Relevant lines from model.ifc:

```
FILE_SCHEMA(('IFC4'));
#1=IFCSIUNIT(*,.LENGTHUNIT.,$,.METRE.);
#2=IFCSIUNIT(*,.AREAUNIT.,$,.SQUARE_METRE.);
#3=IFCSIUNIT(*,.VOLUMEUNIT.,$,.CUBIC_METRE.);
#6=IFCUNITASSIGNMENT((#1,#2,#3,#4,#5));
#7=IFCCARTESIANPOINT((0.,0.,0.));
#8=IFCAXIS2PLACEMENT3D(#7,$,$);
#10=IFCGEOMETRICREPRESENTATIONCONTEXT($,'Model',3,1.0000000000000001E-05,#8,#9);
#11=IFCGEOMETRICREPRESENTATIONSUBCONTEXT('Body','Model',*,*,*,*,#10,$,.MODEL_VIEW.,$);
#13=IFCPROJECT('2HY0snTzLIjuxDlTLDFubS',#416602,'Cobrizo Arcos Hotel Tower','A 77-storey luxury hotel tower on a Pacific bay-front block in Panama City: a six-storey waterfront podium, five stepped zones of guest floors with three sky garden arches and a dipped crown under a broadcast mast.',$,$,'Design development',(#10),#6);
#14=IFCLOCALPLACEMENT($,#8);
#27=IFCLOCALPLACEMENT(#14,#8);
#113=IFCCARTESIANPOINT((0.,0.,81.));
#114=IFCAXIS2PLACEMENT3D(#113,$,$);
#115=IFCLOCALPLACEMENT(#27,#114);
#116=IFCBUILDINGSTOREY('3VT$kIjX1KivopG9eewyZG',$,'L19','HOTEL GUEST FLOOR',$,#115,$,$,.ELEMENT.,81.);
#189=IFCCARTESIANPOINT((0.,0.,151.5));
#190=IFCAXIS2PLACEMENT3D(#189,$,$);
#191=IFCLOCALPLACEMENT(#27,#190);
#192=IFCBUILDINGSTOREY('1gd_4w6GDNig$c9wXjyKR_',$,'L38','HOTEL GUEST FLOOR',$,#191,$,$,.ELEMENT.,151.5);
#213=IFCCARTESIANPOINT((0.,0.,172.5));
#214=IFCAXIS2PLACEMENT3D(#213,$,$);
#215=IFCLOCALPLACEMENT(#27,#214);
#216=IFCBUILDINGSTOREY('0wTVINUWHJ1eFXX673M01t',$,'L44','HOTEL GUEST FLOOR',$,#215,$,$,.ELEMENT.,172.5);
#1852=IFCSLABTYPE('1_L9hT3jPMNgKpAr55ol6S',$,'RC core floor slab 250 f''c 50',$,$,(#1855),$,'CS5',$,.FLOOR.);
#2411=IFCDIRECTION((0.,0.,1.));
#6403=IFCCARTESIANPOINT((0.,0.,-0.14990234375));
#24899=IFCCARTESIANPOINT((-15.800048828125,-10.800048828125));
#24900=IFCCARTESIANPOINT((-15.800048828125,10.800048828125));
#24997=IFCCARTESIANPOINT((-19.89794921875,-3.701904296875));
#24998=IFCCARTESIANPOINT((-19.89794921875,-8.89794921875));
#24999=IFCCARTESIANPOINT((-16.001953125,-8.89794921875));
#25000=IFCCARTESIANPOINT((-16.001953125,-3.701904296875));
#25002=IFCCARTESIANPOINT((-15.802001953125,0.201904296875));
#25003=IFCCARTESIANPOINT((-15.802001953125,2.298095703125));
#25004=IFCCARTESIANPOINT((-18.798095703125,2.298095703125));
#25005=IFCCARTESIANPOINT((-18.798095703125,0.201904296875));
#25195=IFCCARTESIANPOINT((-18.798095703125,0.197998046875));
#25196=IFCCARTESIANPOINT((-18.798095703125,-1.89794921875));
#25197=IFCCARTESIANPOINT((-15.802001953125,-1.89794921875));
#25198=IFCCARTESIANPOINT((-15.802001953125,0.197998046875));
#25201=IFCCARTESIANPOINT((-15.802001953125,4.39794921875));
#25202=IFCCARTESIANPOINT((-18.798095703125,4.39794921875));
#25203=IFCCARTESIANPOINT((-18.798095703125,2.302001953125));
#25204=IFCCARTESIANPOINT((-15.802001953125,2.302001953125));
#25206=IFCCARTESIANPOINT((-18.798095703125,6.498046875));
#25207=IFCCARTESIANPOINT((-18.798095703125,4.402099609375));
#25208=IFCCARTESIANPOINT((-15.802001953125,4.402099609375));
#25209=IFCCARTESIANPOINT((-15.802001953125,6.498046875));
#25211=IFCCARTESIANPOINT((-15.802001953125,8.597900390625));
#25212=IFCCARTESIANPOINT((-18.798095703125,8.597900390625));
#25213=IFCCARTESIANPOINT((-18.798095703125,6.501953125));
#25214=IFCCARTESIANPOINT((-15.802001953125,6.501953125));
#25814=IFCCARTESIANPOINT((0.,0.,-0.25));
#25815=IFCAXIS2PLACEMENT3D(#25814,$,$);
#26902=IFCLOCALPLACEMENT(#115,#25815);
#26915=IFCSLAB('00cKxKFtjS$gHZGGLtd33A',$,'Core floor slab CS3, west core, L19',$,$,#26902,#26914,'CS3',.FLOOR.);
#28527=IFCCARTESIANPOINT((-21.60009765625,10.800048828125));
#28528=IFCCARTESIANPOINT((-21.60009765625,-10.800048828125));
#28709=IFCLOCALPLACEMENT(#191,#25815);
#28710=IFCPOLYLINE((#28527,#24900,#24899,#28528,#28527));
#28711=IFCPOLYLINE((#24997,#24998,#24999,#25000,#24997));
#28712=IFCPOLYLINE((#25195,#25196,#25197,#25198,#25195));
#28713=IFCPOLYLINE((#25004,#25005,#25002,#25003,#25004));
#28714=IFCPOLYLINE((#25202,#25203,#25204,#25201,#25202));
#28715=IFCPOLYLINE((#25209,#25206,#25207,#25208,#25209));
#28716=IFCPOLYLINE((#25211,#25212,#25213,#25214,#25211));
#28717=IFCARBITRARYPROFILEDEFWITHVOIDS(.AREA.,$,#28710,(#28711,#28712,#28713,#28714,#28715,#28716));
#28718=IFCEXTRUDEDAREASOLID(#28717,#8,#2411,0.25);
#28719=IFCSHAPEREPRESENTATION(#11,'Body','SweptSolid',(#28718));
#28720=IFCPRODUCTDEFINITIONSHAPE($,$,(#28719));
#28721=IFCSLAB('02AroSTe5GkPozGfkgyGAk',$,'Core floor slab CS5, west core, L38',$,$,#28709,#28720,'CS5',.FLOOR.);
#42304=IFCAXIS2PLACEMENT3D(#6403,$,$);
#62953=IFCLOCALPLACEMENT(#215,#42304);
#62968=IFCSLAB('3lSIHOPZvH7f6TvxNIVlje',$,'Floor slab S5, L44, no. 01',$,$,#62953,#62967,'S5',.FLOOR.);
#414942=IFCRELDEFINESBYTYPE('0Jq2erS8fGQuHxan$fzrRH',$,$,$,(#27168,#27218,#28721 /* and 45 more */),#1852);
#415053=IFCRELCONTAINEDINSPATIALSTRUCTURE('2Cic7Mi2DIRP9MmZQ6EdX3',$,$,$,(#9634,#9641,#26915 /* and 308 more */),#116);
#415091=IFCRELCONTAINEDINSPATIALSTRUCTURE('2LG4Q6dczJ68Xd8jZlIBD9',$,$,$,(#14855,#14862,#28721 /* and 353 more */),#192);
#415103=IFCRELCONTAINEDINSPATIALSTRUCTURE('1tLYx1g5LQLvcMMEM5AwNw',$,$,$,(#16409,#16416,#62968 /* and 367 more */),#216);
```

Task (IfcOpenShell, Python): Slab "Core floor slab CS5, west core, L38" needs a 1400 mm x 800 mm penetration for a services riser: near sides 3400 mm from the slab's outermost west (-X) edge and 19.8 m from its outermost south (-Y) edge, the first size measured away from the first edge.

```python
import numpy as np
import ifcopenshell
import ifcopenshell.api.feature
import ifcopenshell.api.geometry
import ifcopenshell.api.root
import ifcopenshell.geom
import ifcopenshell.util.placement
import ifcopenshell.util.representation
import ifcopenshell.util.shape
import ifcopenshell.util.unit

model = ifcopenshell.open("model.ifc")
unit_scale = ifcopenshell.util.unit.calculate_unit_scale(model)
settings = ifcopenshell.geom.settings()


def volume(element):
    """Net volume in cubic metres, openings subtracted."""
    shape = ifcopenshell.geom.create_shape(settings, element)
    return ifcopenshell.util.shape.get_volume(shape.geometry)


slab = model.by_id(28721)
before = volume(slab)

# Extent in the slab's own axes, in metres. The edges named are its -X and -Y sides.
slab_shape = ifcopenshell.geom.create_shape(settings, slab)
vertices = ifcopenshell.util.shape.get_vertices(slab_shape.geometry)
x_min, y_min, bottom = vertices.min(axis=0)
top = vertices[:, 2].max()

opening = ifcopenshell.api.root.create_entity(model, ifc_class="IfcOpeningElement", name="Services riser opening", predefined_type="OPENING")
context = ifcopenshell.util.representation.get_context(model, "Model", "Body", "MODEL_VIEW")
width, depth = 1.4, 0.8
outline = [(0.0, 0.0), (width, 0.0), (width, depth), (0.0, depth), (0.0, 0.0)]
# Overshoot both faces by 50 mm so the cut is clean.
shape = ifcopenshell.api.geometry.add_slab_representation(
    model, context=context, depth=top - bottom + 0.1, polyline=outline
)
ifcopenshell.api.geometry.assign_representation(model, product=opening, representation=shape)

matrix = ifcopenshell.util.placement.get_local_placement(slab.ObjectPlacement)
matrix[:, 3] = matrix @ np.append(np.array([x_min + 3.4, y_min + 19.8, bottom - 0.05]) / unit_scale, 1.0)
ifcopenshell.api.geometry.edit_object_placement(model, product=opening, matrix=matrix, is_si=False)
ifcopenshell.api.feature.add_feature(model, feature=opening, element=slab)

after = volume(slab)

print(f"slab volume {before:.3f} -> {after:.3f} m3")

model.write("model_v2.ifc")
```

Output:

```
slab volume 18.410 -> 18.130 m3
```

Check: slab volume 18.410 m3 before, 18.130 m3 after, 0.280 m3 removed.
